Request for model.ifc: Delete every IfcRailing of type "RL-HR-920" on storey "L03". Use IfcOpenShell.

First a look at what the model holds.

```python
import ifcopenshell
import ifcopenshell.util.element

model = ifcopenshell.open("model.ifc")
print(model.schema)
storey = next(s for s in model.by_type("IfcBuildingStorey") if s.Name == "L03")
railings = [e for e in ifcopenshell.util.element.get_decomposition(storey) if e.is_a("IfcRailing")]
seen = {}
for e in railings:
    element_type = ifcopenshell.util.element.get_type(e)
    name = element_type.Name if element_type not in (None, e) else None
    seen[name] = seen.get(name, 0) + 1
for name, count in sorted(seen.items(), key=str):
    print(count, "x", name)
```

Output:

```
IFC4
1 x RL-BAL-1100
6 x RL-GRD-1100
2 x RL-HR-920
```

```python
import ifcopenshell
import ifcopenshell.api.root
import ifcopenshell.util.element

model = ifcopenshell.open("model.ifc")

storey = next(s for s in model.by_type("IfcBuildingStorey") if s.Name == "L03")
railings = [e for e in ifcopenshell.util.element.get_decomposition(storey) if e.is_a("IfcRailing")]
targets = [e for e in railings if (t := ifcopenshell.util.element.get_type(e)) not in (None, e) and t.Name == "RL-HR-920"]

for e in targets:
    ifcopenshell.api.root.remove_product(model, product=e)
print(len(targets), "removed")

model.write("model_v2.ifc")
```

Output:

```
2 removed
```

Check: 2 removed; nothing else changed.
